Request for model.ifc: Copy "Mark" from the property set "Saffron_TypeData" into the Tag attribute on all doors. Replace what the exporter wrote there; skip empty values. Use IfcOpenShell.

First a look at what the model holds.

```python
import ifcopenshell
import ifcopenshell.util.element

model = ifcopenshell.open("model.ifc")
print(model.schema)
doors = model.by_type("IfcDoor")
print(len(doors), "doors")
for e in doors[:8]:
    source = ifcopenshell.util.element.get_pset(e, "Saffron_TypeData", "Mark")
    target = e.Tag
    print(e.id(), repr(source), repr(target), sep=" | ")
```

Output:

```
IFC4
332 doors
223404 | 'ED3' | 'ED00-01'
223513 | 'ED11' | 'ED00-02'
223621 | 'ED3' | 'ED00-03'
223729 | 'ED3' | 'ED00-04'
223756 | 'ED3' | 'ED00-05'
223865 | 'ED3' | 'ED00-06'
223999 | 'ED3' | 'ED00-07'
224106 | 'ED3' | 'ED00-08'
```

```python
import ifcopenshell
import ifcopenshell.util.element

model = ifcopenshell.open("model.ifc")

count = 0
for e in model.by_type("IfcDoor"):
    value = ifcopenshell.util.element.get_pset(e, "Saffron_TypeData", "Mark")
    current = e.Tag
    if not value or not value.strip() or current == value:
        continue
    e.Tag = value
    count += 1

print(count, "doors updated")

model.write("model_rev.ifc")
```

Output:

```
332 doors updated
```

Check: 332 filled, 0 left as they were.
